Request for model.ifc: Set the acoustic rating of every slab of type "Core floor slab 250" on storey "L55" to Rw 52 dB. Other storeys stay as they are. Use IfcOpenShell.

First a look at what the model holds.

```python
import ifcopenshell
import ifcopenshell.util.element

model = ifcopenshell.open("model.ifc")
print(model.schema)
storey = next(s for s in model.by_type("IfcBuildingStorey") if s.Name == "L55")
slabs = [e for e in ifcopenshell.util.element.get_decomposition(storey) if e.is_a("IfcSlab")]
seen = {}
for e in slabs:
    element_type = ifcopenshell.util.element.get_type(e)
    key = (element_type.Name if element_type != e and element_type else None, ifcopenshell.util.element.get_pset(e, "Pset_SlabCommon", "AcousticRating"))
    seen[key] = seen.get(key, 0) + 1
for (name, value), count in sorted(seen.items(), key=str):
    print(count, "x", name, "|", value)
```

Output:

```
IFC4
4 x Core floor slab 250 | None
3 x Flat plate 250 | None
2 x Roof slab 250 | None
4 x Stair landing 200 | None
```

```python
import ifcopenshell
import ifcopenshell.api.pset
import ifcopenshell.util.element

model = ifcopenshell.open("model.ifc")

storey = next(s for s in model.by_type("IfcBuildingStorey") if s.Name == "L55")
slabs = [e for e in ifcopenshell.util.element.get_decomposition(storey) if e.is_a("IfcSlab")]

count = 0
for e in slabs:
    element_type = ifcopenshell.util.element.get_type(e)
    if element_type in (None, e) or element_type.Name != "Core floor slab 250":
        continue
    found = ifcopenshell.util.element.get_pset(e, "Pset_SlabCommon", should_inherit=False)
    if found:
        pset = model.by_id(found["id"])
        if len(ifcopenshell.util.element.get_elements_by_pset(pset)) > 1:
            pset = ifcopenshell.api.pset.unshare_pset(model, products=[e], pset=pset)[0]
    else:
        pset = ifcopenshell.api.pset.add_pset(model, product=e, name="Pset_SlabCommon")
    ifcopenshell.api.pset.edit_pset(model, pset=pset, properties={"AcousticRating": "Rw 52 dB"})
    count += 1

print(count, "slabs updated")

model.write("model-out.ifc")
```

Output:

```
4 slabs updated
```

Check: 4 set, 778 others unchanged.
